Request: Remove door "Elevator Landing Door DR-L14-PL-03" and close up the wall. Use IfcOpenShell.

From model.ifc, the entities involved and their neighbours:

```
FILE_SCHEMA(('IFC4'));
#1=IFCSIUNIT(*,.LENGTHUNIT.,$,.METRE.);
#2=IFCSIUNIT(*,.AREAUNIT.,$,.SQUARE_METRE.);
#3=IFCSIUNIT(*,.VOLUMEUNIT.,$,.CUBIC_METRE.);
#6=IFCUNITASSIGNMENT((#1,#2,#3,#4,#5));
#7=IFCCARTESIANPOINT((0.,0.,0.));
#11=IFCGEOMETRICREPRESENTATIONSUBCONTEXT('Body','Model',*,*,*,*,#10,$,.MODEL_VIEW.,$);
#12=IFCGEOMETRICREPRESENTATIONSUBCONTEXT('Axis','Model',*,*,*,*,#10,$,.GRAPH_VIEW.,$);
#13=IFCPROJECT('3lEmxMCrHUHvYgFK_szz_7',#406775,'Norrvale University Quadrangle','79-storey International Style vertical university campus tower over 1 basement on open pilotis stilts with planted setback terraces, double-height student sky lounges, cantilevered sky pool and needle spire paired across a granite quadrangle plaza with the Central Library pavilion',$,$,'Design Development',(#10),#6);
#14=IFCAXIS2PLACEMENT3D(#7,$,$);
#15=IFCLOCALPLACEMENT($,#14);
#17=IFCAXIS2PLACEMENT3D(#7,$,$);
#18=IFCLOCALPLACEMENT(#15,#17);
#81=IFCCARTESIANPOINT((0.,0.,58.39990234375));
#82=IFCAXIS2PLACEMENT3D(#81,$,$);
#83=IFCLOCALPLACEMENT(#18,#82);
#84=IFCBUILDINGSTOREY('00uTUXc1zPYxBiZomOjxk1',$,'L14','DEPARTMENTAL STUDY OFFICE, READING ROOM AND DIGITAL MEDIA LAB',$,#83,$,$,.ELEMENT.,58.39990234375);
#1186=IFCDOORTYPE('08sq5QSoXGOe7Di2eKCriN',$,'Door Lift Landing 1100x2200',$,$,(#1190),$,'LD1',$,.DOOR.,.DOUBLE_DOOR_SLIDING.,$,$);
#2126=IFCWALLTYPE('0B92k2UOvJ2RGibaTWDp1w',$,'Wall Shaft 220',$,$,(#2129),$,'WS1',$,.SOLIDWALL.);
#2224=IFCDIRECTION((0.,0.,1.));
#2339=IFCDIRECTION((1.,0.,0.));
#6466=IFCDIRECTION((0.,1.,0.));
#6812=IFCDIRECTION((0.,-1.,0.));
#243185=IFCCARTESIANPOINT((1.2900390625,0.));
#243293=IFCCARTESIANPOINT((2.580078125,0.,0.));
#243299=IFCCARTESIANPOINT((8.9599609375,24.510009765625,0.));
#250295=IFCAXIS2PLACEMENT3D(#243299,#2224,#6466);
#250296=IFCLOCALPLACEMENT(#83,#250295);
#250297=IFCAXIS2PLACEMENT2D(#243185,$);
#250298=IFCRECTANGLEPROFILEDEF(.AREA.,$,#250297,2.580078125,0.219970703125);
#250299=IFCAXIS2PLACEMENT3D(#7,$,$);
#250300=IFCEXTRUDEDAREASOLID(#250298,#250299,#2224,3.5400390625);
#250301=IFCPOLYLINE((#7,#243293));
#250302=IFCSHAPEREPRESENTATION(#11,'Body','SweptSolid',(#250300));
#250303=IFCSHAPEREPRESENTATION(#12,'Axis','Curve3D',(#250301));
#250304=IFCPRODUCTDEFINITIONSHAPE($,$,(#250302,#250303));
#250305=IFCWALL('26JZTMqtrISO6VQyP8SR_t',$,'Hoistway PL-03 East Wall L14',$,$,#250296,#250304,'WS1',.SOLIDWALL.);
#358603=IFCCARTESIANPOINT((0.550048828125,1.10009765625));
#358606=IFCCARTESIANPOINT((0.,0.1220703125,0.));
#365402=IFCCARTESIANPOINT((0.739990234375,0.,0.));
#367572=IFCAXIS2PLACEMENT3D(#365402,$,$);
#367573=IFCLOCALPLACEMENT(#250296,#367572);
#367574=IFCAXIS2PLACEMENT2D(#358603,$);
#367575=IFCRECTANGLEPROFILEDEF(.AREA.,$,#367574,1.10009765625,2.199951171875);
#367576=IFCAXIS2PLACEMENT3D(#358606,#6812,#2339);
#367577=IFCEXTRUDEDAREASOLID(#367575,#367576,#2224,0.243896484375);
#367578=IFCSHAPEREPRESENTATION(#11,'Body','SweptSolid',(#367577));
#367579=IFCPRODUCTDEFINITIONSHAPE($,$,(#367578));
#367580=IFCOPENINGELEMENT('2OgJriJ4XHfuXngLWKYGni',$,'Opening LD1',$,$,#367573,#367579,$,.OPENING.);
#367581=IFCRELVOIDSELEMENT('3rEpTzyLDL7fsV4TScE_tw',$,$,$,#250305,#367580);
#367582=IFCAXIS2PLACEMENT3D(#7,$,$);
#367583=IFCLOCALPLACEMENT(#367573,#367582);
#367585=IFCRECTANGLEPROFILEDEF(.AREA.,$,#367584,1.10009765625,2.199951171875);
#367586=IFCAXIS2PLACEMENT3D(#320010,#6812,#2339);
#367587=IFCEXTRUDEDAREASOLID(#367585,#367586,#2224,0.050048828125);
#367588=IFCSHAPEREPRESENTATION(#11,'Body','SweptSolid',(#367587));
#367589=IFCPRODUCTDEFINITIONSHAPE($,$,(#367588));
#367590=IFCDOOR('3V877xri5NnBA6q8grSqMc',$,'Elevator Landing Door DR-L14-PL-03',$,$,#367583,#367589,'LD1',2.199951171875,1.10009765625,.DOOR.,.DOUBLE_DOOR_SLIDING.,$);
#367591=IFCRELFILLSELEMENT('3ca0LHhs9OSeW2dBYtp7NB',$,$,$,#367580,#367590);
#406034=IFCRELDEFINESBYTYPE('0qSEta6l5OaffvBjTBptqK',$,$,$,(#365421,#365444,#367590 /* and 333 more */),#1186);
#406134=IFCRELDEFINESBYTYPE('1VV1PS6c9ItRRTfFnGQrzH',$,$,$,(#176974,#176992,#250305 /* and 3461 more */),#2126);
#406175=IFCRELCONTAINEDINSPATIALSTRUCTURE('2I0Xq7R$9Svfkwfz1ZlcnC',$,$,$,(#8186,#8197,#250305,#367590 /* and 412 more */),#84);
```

```python
import ifcopenshell
import ifcopenshell.api.feature
import ifcopenshell.api.root
import ifcopenshell.geom
import ifcopenshell.util.shape

model = ifcopenshell.open("model.ifc")
settings = ifcopenshell.geom.settings()


def volume(element):
    """Net volume in cubic metres, openings subtracted."""
    shape = ifcopenshell.geom.create_shape(settings, element)
    return ifcopenshell.util.shape.get_volume(shape.geometry)


door = model.by_id(367590)
opening = door.FillsVoids[0].RelatingOpeningElement
wall = opening.VoidsElements[0].RelatingBuildingElement
before = volume(wall)

ifcopenshell.api.root.remove_product(model, product=door)
ifcopenshell.api.feature.remove_feature(model, feature=opening)

after = volume(wall)

print(f"wall volume {before:.3f} -> {after:.3f} m3")

model.write("model-out.ifc")
```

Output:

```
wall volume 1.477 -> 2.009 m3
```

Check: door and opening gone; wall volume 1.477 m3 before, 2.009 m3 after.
